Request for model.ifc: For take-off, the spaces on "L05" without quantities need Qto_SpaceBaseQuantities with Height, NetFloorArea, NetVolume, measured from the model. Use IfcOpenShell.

First a look at what the model holds.

```python
import ifcopenshell
import ifcopenshell.util.element
import ifcopenshell.util.unit

model = ifcopenshell.open("model.ifc")
print(model.schema)
for unit_type in ("LENGTHUNIT", "AREAUNIT", "VOLUMEUNIT"):
    print(unit_type, ifcopenshell.util.unit.calculate_unit_scale(model, unit_type))
storey = next(s for s in model.by_type("IfcBuildingStorey") if s.Name == "L05")
spaces = [e for e in ifcopenshell.util.element.get_decomposition(storey) if e.is_a("IfcSpace")]
for e in sorted(spaces, key=lambda e: e.id()):
    print(e.id(), e.is_a(), e.Name, list(ifcopenshell.util.element.get_psets(e, qtos_only=True)), sep=" | ")
```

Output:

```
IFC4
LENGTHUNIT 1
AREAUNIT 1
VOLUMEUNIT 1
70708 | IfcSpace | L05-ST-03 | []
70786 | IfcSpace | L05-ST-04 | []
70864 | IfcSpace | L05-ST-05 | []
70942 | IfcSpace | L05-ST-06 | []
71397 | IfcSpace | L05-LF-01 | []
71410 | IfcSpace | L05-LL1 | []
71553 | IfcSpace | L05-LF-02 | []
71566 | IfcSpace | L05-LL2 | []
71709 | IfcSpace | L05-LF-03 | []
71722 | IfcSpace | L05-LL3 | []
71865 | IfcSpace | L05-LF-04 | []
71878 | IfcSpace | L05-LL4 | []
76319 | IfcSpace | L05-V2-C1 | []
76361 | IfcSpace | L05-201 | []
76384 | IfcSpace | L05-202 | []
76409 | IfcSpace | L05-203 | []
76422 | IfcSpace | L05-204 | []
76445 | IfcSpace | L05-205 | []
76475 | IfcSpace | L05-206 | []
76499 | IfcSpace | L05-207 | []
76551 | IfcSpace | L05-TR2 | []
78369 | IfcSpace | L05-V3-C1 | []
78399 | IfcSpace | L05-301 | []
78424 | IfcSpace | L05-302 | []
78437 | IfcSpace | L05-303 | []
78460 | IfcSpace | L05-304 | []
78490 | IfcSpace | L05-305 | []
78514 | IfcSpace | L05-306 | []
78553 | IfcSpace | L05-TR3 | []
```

```python
import ifcopenshell
import ifcopenshell.api.pset
import ifcopenshell.geom
import ifcopenshell.util.element
import ifcopenshell.util.shape
import ifcopenshell.util.unit

model = ifcopenshell.open("model.ifc")
unit_scale = ifcopenshell.util.unit.calculate_unit_scale(model)
area_scale = ifcopenshell.util.unit.calculate_unit_scale(model, "AREAUNIT")
volume_scale = ifcopenshell.util.unit.calculate_unit_scale(model, "VOLUMEUNIT")
settings = ifcopenshell.geom.settings()

storey = next(s for s in model.by_type("IfcBuildingStorey") if s.Name == "L05")
spaces = [e for e in ifcopenshell.util.element.get_decomposition(storey) if e.is_a("IfcSpace")]

for e in sorted(spaces, key=lambda e: e.id()):
    if ifcopenshell.util.element.get_psets(e, qtos_only=True, should_inherit=False):
        continue
    # Geometry comes back in metres, in the element's own axes.
    shape = ifcopenshell.geom.create_shape(settings, e)
    values = {
        "Height": ifcopenshell.util.shape.get_z(shape.geometry) / unit_scale,
        "NetFloorArea": ifcopenshell.util.shape.get_footprint_area(shape.geometry) / area_scale,
        "NetVolume": ifcopenshell.util.shape.get_volume(shape.geometry) / volume_scale,
    }
    qto = ifcopenshell.api.pset.add_qto(model, product=e, name="Qto_SpaceBaseQuantities")
    ifcopenshell.api.pset.edit_qto(model, qto=qto, properties=values)
    print(e.id(), {k: round(v, 3) for k, v in values.items()})

model.write("model_rev.ifc")
```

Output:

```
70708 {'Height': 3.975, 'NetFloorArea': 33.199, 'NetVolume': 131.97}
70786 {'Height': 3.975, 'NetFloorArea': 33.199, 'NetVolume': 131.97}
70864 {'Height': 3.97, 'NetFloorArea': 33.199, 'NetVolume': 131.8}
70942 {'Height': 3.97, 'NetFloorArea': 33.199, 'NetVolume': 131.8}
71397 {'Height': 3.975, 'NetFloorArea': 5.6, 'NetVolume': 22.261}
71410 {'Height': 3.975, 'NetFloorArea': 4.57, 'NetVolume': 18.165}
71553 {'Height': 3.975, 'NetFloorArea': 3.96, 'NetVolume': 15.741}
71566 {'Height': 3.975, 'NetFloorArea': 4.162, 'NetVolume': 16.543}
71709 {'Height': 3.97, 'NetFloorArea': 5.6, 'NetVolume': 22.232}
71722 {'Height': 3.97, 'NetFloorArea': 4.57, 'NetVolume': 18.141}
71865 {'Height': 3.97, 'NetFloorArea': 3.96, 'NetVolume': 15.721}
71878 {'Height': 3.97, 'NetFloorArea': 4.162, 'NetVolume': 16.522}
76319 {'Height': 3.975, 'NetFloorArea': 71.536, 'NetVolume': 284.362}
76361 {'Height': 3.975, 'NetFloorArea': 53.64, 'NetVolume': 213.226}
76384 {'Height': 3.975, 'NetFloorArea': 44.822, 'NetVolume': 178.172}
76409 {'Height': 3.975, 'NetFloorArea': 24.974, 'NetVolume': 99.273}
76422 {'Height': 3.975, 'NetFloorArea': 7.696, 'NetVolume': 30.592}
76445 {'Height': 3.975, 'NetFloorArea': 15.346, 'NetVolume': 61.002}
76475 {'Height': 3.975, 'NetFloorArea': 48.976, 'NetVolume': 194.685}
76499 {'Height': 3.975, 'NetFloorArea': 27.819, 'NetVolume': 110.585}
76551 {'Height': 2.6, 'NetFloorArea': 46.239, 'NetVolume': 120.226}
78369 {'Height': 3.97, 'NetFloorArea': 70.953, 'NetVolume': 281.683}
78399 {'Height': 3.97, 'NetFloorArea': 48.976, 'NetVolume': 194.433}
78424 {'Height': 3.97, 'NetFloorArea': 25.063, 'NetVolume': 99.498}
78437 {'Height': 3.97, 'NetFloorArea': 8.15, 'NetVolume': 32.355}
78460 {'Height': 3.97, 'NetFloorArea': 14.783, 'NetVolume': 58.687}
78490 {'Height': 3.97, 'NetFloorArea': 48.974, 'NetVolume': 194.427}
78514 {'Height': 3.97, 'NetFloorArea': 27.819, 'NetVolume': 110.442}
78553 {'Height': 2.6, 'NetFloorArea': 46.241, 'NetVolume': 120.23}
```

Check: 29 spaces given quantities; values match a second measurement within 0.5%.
